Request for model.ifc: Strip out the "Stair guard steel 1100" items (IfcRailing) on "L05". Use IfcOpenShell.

First a look at what the model holds.

```python
import ifcopenshell
import ifcopenshell.util.element

model = ifcopenshell.open("model.ifc")
print(model.schema)
storey = next(s for s in model.by_type("IfcBuildingStorey") if s.Name == "L05")
railings = [e for e in ifcopenshell.util.element.get_decomposition(storey) if e.is_a("IfcRailing")]
seen = {}
for e in railings:
    element_type = ifcopenshell.util.element.get_type(e)
    name = element_type.Name if element_type not in (None, e) else None
    seen[name] = seen.get(name, 0) + 1
for name, count in sorted(seen.items(), key=str):
    print(count, "x", name)
```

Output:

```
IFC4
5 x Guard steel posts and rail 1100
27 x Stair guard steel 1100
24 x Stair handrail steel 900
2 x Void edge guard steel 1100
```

```python
import ifcopenshell
import ifcopenshell.api.root
import ifcopenshell.util.element

model = ifcopenshell.open("model.ifc")

storey = next(s for s in model.by_type("IfcBuildingStorey") if s.Name == "L05")
railings = [e for e in ifcopenshell.util.element.get_decomposition(storey) if e.is_a("IfcRailing")]
targets = [e for e in railings if (t := ifcopenshell.util.element.get_type(e)) not in (None, e) and t.Name == "Stair guard steel 1100"]

for e in targets:
    ifcopenshell.api.root.remove_product(model, product=e)
print(len(targets), "removed")

model.write("model_v2.ifc")
```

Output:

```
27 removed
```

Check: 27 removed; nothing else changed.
